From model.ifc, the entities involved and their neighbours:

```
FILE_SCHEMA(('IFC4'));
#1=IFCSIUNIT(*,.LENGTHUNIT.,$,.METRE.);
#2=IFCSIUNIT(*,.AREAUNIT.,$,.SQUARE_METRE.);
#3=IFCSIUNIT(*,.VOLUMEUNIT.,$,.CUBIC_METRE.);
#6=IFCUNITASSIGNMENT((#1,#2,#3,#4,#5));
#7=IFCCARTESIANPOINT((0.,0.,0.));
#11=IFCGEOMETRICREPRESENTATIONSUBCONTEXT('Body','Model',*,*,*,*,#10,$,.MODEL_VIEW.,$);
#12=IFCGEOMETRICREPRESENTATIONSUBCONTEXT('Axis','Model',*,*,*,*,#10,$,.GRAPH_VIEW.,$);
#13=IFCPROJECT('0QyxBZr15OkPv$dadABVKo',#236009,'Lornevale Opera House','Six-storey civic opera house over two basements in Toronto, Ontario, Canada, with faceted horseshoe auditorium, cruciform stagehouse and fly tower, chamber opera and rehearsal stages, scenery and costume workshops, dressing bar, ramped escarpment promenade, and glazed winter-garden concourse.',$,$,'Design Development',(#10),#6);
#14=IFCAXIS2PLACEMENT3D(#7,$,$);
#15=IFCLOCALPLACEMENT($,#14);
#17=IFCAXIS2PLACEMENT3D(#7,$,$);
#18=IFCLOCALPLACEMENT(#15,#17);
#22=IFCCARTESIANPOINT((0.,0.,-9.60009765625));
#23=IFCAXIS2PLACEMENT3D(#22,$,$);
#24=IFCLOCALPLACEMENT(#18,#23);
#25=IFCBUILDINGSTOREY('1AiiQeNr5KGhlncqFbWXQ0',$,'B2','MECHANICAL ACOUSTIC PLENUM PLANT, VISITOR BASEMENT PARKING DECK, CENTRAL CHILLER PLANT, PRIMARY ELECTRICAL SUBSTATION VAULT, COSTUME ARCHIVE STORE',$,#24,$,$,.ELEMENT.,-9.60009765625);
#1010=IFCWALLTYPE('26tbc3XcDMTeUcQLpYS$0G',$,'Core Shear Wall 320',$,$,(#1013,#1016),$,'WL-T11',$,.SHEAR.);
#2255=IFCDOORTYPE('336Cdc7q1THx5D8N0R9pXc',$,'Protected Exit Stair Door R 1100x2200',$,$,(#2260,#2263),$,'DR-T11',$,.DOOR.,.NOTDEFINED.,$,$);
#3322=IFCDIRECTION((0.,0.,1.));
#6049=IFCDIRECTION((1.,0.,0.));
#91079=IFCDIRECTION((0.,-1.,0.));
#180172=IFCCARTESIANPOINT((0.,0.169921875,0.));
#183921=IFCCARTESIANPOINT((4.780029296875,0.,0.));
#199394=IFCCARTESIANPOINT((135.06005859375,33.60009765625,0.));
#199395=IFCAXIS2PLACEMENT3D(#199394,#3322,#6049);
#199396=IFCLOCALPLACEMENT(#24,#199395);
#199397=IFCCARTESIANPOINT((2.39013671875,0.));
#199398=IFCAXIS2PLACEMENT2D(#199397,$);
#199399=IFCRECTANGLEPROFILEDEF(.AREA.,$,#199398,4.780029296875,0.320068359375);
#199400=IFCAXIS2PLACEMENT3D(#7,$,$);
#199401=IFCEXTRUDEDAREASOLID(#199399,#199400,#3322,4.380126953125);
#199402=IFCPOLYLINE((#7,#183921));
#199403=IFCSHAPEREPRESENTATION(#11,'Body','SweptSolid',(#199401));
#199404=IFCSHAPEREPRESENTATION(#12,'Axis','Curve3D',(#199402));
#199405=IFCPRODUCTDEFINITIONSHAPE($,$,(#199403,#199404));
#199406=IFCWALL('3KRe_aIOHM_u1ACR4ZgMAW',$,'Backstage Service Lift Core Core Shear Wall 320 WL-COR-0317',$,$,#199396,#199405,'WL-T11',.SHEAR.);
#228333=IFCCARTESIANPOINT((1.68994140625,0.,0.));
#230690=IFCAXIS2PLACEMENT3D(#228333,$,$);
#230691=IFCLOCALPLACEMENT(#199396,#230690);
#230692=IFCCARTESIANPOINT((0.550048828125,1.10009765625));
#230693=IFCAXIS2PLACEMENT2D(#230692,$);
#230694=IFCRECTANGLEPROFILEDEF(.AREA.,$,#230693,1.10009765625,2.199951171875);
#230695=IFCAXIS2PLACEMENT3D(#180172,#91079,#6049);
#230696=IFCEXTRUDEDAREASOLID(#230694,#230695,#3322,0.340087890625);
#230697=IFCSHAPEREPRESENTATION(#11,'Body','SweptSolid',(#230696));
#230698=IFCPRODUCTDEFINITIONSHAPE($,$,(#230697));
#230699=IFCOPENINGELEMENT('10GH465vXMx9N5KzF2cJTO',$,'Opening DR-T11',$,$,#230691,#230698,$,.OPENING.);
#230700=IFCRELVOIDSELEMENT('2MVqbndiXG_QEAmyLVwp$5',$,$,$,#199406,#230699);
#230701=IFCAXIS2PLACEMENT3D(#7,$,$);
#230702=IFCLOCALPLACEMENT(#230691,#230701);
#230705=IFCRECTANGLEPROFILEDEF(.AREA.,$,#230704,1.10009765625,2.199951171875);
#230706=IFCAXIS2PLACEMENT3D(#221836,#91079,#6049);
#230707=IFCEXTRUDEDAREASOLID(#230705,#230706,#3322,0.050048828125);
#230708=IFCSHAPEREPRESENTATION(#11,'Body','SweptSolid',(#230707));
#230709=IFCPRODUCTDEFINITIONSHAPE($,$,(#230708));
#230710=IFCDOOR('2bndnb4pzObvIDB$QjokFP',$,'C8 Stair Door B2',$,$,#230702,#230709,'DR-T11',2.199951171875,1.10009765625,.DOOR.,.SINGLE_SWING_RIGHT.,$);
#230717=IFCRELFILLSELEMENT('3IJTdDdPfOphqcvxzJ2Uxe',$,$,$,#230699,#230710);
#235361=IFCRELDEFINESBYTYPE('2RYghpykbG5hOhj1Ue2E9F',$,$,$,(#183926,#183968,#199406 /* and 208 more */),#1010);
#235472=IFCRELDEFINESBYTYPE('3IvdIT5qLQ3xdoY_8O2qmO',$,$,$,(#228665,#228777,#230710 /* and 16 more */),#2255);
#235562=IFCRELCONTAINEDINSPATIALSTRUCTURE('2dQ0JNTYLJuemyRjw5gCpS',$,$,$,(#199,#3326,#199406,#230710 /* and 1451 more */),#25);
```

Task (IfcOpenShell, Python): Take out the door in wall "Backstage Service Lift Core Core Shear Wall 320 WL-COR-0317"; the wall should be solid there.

```python
import ifcopenshell
import ifcopenshell.api.feature
import ifcopenshell.api.root
import ifcopenshell.geom
import ifcopenshell.util.shape

model = ifcopenshell.open("model.ifc")
settings = ifcopenshell.geom.settings()


def volume(element):
    """Net volume in cubic metres, openings subtracted."""
    shape = ifcopenshell.geom.create_shape(settings, element)
    return ifcopenshell.util.shape.get_volume(shape.geometry)


door = model.by_guid("2bndnb4pzObvIDB$QjokFP")
opening = door.FillsVoids[0].RelatingOpeningElement
wall = opening.VoidsElements[0].RelatingBuildingElement
before = volume(wall)

ifcopenshell.api.root.remove_product(model, product=door)
ifcopenshell.api.feature.remove_feature(model, feature=opening)

after = volume(wall)

print(f"wall volume {before:.3f} -> {after:.3f} m3")

model.write("model-out.ifc")
```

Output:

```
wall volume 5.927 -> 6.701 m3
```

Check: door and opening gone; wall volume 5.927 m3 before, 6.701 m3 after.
